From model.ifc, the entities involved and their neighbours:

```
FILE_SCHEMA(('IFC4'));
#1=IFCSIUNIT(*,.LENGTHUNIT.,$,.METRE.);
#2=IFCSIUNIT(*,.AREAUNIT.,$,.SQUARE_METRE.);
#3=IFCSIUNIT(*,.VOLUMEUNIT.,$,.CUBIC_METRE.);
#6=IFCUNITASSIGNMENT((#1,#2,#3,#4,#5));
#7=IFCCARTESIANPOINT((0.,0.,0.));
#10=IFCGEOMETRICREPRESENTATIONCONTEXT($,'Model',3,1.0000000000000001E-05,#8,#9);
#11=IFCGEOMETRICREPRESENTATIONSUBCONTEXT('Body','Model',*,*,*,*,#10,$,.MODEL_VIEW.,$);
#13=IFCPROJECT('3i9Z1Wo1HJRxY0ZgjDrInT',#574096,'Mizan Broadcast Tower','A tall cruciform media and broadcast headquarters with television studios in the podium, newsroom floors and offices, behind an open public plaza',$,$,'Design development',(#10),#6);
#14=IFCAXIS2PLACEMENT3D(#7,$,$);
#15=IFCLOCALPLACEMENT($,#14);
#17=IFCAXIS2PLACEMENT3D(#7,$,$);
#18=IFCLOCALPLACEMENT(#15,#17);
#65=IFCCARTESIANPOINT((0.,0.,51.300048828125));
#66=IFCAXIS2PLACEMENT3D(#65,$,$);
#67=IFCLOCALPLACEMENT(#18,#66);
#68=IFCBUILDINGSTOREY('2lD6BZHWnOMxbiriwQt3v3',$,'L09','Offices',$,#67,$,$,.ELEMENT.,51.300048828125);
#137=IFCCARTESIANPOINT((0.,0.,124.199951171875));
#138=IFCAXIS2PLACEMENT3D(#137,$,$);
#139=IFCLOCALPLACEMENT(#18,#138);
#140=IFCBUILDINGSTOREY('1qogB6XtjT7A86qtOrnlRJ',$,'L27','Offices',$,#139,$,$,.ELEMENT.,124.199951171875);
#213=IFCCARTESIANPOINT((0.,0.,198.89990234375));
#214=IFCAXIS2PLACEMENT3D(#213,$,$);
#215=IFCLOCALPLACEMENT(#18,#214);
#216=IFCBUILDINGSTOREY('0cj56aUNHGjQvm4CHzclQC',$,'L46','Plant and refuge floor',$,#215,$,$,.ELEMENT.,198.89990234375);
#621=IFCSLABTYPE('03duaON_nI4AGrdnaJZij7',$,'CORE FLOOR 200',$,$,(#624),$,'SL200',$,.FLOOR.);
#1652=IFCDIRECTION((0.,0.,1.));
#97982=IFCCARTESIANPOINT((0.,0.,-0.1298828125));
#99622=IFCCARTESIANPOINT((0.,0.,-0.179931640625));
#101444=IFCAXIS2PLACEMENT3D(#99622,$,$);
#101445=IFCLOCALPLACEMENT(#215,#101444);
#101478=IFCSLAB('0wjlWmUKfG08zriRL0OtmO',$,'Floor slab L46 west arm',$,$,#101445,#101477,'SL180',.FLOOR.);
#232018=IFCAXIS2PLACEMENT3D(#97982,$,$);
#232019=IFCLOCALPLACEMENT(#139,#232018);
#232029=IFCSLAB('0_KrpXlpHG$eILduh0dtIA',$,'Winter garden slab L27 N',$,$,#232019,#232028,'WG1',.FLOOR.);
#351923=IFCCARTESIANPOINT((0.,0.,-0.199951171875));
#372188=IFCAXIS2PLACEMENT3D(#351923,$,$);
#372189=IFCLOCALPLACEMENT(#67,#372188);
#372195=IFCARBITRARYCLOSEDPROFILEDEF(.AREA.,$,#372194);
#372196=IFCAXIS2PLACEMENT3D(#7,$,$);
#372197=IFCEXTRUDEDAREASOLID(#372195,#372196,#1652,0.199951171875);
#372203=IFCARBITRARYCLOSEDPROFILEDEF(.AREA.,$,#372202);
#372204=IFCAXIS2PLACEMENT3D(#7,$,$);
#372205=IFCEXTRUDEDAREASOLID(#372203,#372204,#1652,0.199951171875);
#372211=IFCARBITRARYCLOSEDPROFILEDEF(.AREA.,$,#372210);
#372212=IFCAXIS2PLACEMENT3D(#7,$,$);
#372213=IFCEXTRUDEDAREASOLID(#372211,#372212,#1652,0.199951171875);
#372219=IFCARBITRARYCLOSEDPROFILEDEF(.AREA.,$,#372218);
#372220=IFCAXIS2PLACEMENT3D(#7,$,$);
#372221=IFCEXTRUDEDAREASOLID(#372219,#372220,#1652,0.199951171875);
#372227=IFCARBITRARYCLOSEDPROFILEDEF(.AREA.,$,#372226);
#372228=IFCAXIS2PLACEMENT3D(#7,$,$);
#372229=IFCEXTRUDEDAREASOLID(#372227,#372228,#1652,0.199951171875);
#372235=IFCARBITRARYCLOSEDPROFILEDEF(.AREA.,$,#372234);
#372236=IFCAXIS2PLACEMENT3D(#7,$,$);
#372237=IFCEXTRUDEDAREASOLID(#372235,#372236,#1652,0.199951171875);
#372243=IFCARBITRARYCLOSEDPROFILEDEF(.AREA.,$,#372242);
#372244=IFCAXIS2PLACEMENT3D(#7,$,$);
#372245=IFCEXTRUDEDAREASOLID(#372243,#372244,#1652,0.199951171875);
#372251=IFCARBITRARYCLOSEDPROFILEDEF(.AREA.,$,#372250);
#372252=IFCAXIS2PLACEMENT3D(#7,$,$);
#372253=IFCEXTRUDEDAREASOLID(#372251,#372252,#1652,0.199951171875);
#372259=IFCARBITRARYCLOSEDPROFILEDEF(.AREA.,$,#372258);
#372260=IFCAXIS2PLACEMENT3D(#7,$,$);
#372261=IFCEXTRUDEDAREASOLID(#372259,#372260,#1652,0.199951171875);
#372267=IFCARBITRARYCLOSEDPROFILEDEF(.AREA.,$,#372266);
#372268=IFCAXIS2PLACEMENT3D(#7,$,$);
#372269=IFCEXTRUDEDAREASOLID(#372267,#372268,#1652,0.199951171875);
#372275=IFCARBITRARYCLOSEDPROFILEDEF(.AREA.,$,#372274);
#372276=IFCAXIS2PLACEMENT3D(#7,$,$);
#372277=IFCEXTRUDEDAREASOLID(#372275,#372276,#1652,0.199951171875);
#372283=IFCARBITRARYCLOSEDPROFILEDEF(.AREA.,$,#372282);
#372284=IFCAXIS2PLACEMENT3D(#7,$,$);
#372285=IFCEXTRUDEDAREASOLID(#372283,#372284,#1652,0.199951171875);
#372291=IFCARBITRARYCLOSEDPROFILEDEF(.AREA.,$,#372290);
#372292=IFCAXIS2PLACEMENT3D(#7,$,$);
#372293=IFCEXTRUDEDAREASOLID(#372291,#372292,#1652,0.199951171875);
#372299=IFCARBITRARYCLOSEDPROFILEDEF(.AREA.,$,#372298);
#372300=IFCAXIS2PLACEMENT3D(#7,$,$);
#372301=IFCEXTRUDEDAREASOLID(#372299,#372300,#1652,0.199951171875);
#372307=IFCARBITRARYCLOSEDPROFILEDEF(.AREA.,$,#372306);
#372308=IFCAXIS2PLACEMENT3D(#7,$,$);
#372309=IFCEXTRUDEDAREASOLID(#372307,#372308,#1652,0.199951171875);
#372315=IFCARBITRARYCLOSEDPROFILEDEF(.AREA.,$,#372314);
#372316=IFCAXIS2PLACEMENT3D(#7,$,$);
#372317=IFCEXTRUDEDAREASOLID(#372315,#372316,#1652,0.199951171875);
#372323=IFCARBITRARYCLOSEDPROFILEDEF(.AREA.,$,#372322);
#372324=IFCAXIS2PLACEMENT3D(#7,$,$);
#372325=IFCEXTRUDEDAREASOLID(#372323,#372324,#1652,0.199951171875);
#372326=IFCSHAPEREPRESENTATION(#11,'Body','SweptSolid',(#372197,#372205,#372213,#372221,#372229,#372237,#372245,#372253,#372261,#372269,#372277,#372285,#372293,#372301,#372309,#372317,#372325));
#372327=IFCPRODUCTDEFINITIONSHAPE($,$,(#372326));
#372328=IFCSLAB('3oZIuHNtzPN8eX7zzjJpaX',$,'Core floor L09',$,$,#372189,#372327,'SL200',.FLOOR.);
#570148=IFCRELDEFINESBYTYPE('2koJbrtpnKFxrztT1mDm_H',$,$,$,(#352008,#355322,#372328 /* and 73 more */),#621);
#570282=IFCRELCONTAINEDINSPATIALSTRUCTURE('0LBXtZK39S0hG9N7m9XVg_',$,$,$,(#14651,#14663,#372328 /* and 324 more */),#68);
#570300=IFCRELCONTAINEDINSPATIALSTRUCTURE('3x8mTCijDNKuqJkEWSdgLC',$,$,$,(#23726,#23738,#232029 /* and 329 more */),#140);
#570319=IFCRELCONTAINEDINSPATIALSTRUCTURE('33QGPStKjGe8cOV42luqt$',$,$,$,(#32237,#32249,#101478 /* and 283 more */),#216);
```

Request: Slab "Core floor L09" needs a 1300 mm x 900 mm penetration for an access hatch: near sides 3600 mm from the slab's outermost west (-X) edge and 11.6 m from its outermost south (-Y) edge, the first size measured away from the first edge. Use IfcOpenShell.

```python
import numpy as np
import ifcopenshell
import ifcopenshell.api.feature
import ifcopenshell.api.geometry
import ifcopenshell.api.root
import ifcopenshell.geom
import ifcopenshell.util.placement
import ifcopenshell.util.representation
import ifcopenshell.util.shape
import ifcopenshell.util.unit

model = ifcopenshell.open("model.ifc")
unit_scale = ifcopenshell.util.unit.calculate_unit_scale(model)
settings = ifcopenshell.geom.settings()


def volume(element):
    """Net volume in cubic metres, openings subtracted."""
    shape = ifcopenshell.geom.create_shape(settings, element)
    return ifcopenshell.util.shape.get_volume(shape.geometry)


slab = model.by_id(372328)
before = volume(slab)

# Extent in the slab's own axes, in metres. The edges named are its -X and -Y sides.
slab_shape = ifcopenshell.geom.create_shape(settings, slab)
vertices = ifcopenshell.util.shape.get_vertices(slab_shape.geometry)
x_min, y_min, bottom = vertices.min(axis=0)
top = vertices[:, 2].max()

opening = ifcopenshell.api.root.create_entity(model, ifc_class="IfcOpeningElement", name="Access hatch opening", predefined_type="OPENING")
context = ifcopenshell.util.representation.get_context(model, "Model", "Body", "MODEL_VIEW")
width, depth = 1.3, 0.9
outline = [(0.0, 0.0), (width, 0.0), (width, depth), (0.0, depth), (0.0, 0.0)]
# Overshoot both faces by 50 mm so the cut is clean.
shape = ifcopenshell.api.geometry.add_slab_representation(
    model, context=context, depth=top - bottom + 0.1, polyline=outline
)
ifcopenshell.api.geometry.assign_representation(model, product=opening, representation=shape)

matrix = ifcopenshell.util.placement.get_local_placement(slab.ObjectPlacement)
matrix[:, 3] = matrix @ np.append(np.array([x_min + 3.6, y_min + 11.6, bottom - 0.05]) / unit_scale, 1.0)
ifcopenshell.api.geometry.edit_object_placement(model, product=opening, matrix=matrix, is_si=False)
ifcopenshell.api.feature.add_feature(model, feature=opening, element=slab)

after = volume(slab)

print(f"slab volume {before:.3f} -> {after:.3f} m3")

model.write("model_v2.ifc")
```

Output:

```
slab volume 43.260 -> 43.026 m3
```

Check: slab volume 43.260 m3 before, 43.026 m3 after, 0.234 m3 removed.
